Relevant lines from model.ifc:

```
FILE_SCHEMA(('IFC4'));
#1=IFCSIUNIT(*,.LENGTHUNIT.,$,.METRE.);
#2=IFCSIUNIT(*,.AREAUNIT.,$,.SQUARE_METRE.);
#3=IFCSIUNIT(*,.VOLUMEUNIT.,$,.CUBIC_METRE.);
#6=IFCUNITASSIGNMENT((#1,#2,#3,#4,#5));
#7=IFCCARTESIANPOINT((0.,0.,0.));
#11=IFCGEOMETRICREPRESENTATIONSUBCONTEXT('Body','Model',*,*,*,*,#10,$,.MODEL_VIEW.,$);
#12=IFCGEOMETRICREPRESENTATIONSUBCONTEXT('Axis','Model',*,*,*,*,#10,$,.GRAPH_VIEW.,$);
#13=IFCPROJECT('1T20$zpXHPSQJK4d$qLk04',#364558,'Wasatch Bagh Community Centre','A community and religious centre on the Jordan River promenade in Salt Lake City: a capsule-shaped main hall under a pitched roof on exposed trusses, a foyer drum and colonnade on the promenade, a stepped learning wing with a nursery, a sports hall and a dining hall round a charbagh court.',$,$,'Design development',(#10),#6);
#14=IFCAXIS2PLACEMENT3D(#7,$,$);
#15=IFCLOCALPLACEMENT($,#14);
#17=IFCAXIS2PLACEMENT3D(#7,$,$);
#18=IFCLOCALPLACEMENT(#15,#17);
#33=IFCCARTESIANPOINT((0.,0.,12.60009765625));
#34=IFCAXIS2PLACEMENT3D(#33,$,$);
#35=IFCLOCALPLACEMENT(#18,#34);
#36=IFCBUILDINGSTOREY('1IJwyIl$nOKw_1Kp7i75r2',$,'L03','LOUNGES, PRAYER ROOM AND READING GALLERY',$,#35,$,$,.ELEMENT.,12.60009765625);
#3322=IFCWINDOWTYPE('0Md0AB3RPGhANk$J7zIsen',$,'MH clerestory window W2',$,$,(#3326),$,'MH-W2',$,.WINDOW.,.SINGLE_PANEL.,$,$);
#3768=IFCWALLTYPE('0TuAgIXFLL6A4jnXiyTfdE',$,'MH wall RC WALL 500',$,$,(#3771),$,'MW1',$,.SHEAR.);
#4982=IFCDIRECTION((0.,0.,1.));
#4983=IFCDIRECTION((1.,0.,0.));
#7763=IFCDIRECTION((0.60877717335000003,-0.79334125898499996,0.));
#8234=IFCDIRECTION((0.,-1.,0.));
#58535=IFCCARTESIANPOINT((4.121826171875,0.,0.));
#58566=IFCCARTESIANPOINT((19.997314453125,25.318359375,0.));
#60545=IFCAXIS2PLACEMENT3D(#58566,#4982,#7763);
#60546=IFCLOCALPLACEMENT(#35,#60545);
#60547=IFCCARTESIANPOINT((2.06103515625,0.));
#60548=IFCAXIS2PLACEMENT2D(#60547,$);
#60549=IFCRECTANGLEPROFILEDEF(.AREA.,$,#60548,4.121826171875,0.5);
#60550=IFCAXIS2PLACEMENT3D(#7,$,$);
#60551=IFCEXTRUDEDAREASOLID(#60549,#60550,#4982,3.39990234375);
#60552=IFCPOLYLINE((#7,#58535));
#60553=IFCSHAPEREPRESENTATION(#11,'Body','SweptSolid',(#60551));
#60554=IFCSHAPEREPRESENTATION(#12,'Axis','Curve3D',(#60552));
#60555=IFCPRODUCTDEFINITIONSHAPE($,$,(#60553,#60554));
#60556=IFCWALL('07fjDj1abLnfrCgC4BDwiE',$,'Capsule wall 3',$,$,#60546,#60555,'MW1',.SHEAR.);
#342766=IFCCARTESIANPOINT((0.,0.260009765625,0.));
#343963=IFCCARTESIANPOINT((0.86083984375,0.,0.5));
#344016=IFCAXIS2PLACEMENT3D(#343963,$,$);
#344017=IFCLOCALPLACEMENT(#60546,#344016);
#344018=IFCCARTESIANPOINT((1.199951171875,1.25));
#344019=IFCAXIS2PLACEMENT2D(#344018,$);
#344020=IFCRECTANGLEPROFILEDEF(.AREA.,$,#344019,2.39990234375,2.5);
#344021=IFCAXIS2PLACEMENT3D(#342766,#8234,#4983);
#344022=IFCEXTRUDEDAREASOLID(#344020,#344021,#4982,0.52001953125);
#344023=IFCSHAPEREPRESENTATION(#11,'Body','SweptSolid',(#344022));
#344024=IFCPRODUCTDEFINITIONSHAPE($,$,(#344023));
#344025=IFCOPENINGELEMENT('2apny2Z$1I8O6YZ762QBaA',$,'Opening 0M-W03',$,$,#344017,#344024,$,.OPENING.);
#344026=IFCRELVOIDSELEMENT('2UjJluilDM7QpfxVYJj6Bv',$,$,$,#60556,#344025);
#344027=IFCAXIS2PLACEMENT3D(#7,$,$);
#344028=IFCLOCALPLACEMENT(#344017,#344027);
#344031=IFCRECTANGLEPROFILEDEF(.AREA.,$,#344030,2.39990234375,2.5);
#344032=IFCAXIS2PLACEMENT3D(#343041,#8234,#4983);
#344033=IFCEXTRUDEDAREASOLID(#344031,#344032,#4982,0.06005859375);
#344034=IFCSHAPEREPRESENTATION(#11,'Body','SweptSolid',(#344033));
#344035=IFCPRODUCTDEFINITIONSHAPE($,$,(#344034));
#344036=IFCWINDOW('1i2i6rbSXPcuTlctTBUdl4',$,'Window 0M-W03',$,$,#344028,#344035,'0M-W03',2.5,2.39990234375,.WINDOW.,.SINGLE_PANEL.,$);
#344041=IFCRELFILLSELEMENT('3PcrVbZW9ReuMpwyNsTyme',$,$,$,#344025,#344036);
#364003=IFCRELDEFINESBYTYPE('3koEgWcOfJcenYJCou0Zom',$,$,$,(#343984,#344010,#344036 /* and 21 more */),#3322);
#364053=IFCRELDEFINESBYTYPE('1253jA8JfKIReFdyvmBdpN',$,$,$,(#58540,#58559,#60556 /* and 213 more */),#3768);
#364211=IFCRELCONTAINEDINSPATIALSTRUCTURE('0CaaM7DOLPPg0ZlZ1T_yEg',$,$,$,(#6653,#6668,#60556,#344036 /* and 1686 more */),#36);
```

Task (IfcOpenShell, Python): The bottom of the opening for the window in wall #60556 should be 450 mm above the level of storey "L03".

```python
import numpy as np
import ifcopenshell
import ifcopenshell.api.geometry
import ifcopenshell.geom
import ifcopenshell.util.element
import ifcopenshell.util.placement
import ifcopenshell.util.shape
import ifcopenshell.util.unit

model = ifcopenshell.open("model.ifc")
unit_scale = ifcopenshell.util.unit.calculate_unit_scale(model)

window = model.by_id(344036)
opening = window.FillsVoids[0].RelatingOpeningElement
storey = ifcopenshell.util.element.get_container(window, ifc_class="IfcBuildingStorey")
level = ifcopenshell.util.placement.get_local_placement(storey.ObjectPlacement)[2, 3]

# The opening's origin need not be at the sill, so measure its lowest point.
shape = ifcopenshell.geom.create_shape(ifcopenshell.geom.settings(), opening)
bottom = ifcopenshell.util.shape.get_shape_bottom_elevation(shape, shape.geometry) / unit_scale
dz = level + 0.45 / unit_scale - bottom

shift = np.array([0.0, 0.0, dz])
# The window is placed relative to its opening, so it follows when the opening moves.
matrix = ifcopenshell.util.placement.get_local_placement(opening.ObjectPlacement)
matrix[:3, 3] += shift
ifcopenshell.api.geometry.edit_object_placement(
    model, product=opening, matrix=matrix, is_si=False, should_transform_children=True
)

print(f"moved by {dz * unit_scale:+.3f} m")

model.write("model_v2.ifc")
```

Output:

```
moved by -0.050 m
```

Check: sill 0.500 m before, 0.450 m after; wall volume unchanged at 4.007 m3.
